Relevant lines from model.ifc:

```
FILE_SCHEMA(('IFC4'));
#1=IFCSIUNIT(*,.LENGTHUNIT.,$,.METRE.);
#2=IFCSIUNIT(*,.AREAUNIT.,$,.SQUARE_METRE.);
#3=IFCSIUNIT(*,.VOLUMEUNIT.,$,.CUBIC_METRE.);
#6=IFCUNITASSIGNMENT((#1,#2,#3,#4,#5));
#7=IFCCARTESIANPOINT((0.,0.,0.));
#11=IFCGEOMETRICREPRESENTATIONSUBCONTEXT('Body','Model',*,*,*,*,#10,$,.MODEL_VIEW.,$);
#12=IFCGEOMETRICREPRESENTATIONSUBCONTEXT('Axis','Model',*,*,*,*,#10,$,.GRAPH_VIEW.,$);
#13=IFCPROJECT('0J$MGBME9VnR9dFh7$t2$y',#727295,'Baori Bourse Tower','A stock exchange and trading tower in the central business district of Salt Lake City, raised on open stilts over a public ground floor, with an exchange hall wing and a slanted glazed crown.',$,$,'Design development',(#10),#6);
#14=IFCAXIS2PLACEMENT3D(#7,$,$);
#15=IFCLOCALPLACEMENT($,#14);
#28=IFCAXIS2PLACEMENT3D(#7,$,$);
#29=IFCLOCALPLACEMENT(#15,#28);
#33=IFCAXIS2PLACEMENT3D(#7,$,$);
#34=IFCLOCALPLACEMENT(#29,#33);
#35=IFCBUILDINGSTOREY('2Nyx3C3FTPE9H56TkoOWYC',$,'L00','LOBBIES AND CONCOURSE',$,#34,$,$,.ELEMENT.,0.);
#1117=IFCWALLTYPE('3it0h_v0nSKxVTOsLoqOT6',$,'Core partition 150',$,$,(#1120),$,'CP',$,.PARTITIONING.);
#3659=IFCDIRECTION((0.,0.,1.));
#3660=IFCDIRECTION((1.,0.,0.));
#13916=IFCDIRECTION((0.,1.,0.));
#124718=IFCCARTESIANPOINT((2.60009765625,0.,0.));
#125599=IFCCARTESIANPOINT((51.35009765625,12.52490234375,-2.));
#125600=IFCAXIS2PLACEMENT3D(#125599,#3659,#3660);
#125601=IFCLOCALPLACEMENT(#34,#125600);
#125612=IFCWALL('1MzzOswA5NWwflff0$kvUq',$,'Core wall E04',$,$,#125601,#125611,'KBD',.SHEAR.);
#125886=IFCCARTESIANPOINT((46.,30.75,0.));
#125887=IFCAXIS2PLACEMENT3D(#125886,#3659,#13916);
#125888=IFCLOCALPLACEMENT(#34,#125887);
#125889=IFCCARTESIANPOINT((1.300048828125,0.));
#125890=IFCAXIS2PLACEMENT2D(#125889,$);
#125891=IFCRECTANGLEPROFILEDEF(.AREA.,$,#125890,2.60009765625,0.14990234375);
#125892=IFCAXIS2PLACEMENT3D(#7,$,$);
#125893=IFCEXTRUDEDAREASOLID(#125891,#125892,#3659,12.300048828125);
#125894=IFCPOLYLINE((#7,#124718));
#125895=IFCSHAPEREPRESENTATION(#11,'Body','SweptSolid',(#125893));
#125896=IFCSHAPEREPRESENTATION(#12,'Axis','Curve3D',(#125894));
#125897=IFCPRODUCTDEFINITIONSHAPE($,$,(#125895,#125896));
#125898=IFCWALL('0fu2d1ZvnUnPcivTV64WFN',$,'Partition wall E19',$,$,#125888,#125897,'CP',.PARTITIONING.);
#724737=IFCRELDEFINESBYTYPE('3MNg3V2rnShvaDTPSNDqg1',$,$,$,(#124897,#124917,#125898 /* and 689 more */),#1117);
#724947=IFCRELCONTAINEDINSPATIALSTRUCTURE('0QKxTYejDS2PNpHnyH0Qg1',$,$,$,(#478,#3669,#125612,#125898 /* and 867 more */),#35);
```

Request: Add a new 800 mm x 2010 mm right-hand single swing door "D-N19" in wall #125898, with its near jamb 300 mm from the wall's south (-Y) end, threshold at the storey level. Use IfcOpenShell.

```python
import numpy as np
import ifcopenshell
import ifcopenshell.api.feature
import ifcopenshell.api.geometry
import ifcopenshell.api.root
import ifcopenshell.api.spatial
import ifcopenshell.geom
import ifcopenshell.util.element
import ifcopenshell.util.placement
import ifcopenshell.util.representation
import ifcopenshell.util.shape
import ifcopenshell.util.unit

model = ifcopenshell.open("model.ifc")
unit_scale = ifcopenshell.util.unit.calculate_unit_scale(model)
settings = ifcopenshell.geom.settings()


def volume(element):
    """Net volume in cubic metres, openings subtracted."""
    shape = ifcopenshell.geom.create_shape(settings, element)
    return ifcopenshell.util.shape.get_volume(shape.geometry)


wall = model.by_guid("0fu2d1ZvnUnPcivTV64WFN")
storey = ifcopenshell.util.element.get_container(wall, ifc_class="IfcBuildingStorey")
context = ifcopenshell.util.representation.get_context(model, "Model", "Body", "MODEL_VIEW")
before = volume(wall)

width, height, from_end, sill = 0.8, 2.01, 0.3, 0.0  # metres

# The wall runs along its own X axis, and the end named is its -X end.
wall_shape = ifcopenshell.geom.create_shape(settings, wall)
x, y, z = ifcopenshell.util.shape.get_vertices(wall_shape.geometry).T
start = x.min() + from_end
face, thickness = float(y.min()), float(y.max() - y.min())
wall_matrix = ifcopenshell.util.placement.get_local_placement(wall.ObjectPlacement)
level = ifcopenshell.util.placement.get_local_placement(storey.ObjectPlacement)[2, 3]


def in_wall(x, y):
    """Placement at x, y metres in the wall's axes, at sill height."""
    matrix = wall_matrix.copy()
    matrix[:, 3] = wall_matrix @ np.array([x / unit_scale, y / unit_scale, 0.0, 1.0])
    matrix[2, 3] = level + sill / unit_scale
    return matrix


# Opening: a box that overshoots both wall faces by 50 mm.
opening = ifcopenshell.api.root.create_entity(model, ifc_class="IfcOpeningElement", predefined_type="OPENING")
box = ifcopenshell.api.geometry.add_wall_representation(
    model, context=context, length=width, height=height, thickness=thickness + 0.1
)
ifcopenshell.api.geometry.assign_representation(model, product=opening, representation=box)
ifcopenshell.api.geometry.edit_object_placement(model, product=opening, matrix=in_wall(start, face - 0.05), is_si=False)
ifcopenshell.api.feature.add_feature(model, feature=opening, element=wall)

door = ifcopenshell.api.root.create_entity(model, ifc_class="IfcDoor", name="D-N19", predefined_type="DOOR")
door.OverallWidth, door.OverallHeight = width / unit_scale, height / unit_scale
door.OperationType = "SINGLE_SWING_RIGHT"
body = ifcopenshell.api.geometry.add_door_representation(
    model,
    context=context,
    overall_width=door.OverallWidth,
    overall_height=door.OverallHeight,
    operation_type="SINGLE_SWING_RIGHT",
    lining_properties={"LiningDepth": thickness / unit_scale, "ThresholdDepth": thickness / unit_scale},
)
ifcopenshell.api.geometry.assign_representation(model, product=door, representation=body)
ifcopenshell.api.spatial.assign_container(model, products=[door], relating_structure=storey)
ifcopenshell.api.feature.add_filling(model, opening=opening, element=door)

# The lining spans the wall, so the door starts at the wall face.
ifcopenshell.api.geometry.edit_object_placement(model, product=door, matrix=in_wall(start, face), is_si=False)

after = volume(wall)

print(f"wall volume {before:.3f} -> {after:.3f} m3")

model.write("model-out.ifc")
```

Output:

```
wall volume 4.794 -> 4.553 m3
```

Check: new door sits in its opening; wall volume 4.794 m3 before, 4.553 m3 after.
